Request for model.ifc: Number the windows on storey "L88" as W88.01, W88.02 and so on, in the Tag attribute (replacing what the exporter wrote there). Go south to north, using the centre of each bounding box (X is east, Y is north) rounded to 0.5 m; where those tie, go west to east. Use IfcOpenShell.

First a look at what the model holds.

```python
import ifcopenshell
import ifcopenshell.util.element
import ifcopenshell.util.placement

model = ifcopenshell.open("model.ifc")
print(model.schema)
storey = next(s for s in model.by_type("IfcBuildingStorey") if s.Name == "L88")
windows = [e for e in ifcopenshell.util.element.get_decomposition(storey) if e.is_a("IfcWindow")]
for e in sorted(windows, key=lambda e: e.id()):
    origin = ifcopenshell.util.placement.get_local_placement(e.ObjectPlacement)[:3, 3]
    print(e.id(), e.Tag, e.Name, origin.round(2) + 0.0, sep=" | ")
```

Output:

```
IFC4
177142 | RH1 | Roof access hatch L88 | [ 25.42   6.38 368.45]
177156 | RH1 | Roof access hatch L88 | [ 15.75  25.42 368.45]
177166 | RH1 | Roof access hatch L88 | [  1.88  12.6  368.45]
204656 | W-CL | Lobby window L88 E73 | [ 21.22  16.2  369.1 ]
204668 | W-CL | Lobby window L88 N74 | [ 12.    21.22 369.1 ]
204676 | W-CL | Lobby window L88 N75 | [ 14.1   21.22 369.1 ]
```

```python
import ifcopenshell
import ifcopenshell.geom
import ifcopenshell.util.element
import ifcopenshell.util.shape

model = ifcopenshell.open("model.ifc")
settings = ifcopenshell.geom.settings()
settings.set("use-world-coords", True)


def centre(element):
    shape = ifcopenshell.geom.create_shape(settings, element)
    return ifcopenshell.util.shape.get_bbox_centroid(shape.geometry)


storey = next(s for s in model.by_type("IfcBuildingStorey") if s.Name == "L88")
windows = [e for e in ifcopenshell.util.element.get_decomposition(storey) if e.is_a("IfcWindow")]

# Insertion points can sit at a corner or the storey origin, so sort by the geometry (in metres).
centres = {e: centre(e) for e in windows}
windows.sort(key=lambda e: (round(centres[e][1] / 0.5), centres[e][0]))

for i, e in enumerate(windows, start=1):
    number = f"W88.{i:02d}"
    e.Tag = number
    print(e.id(), number)

model.write("model_edited.ifc")
```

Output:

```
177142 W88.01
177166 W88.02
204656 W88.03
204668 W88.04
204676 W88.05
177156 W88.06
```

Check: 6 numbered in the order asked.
